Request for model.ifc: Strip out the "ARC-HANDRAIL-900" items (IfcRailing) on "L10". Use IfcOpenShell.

First a look at what the model holds.

```python
import ifcopenshell
import ifcopenshell.util.element

model = ifcopenshell.open("model.ifc")
print(model.schema)
storey = next(s for s in model.by_type("IfcBuildingStorey") if s.Name == "L10")
railings = [e for e in ifcopenshell.util.element.get_decomposition(storey) if e.is_a("IfcRailing")]
seen = {}
for e in railings:
    element_type = ifcopenshell.util.element.get_type(e)
    name = element_type.Name if element_type not in (None, e) else None
    seen[name] = seen.get(name, 0) + 1
for name, count in sorted(seen.items(), key=str):
    print(count, "x", name)
```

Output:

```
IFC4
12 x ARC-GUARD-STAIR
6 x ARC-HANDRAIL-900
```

```python
import ifcopenshell
import ifcopenshell.api.root
import ifcopenshell.util.element

model = ifcopenshell.open("model.ifc")

storey = next(s for s in model.by_type("IfcBuildingStorey") if s.Name == "L10")
railings = [e for e in ifcopenshell.util.element.get_decomposition(storey) if e.is_a("IfcRailing")]
targets = [e for e in railings if (t := ifcopenshell.util.element.get_type(e)) not in (None, e) and t.Name == "ARC-HANDRAIL-900"]

for e in targets:
    ifcopenshell.api.root.remove_product(model, product=e)
print(len(targets), "removed")

model.write("model_edited.ifc")
```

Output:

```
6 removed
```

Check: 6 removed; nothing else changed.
